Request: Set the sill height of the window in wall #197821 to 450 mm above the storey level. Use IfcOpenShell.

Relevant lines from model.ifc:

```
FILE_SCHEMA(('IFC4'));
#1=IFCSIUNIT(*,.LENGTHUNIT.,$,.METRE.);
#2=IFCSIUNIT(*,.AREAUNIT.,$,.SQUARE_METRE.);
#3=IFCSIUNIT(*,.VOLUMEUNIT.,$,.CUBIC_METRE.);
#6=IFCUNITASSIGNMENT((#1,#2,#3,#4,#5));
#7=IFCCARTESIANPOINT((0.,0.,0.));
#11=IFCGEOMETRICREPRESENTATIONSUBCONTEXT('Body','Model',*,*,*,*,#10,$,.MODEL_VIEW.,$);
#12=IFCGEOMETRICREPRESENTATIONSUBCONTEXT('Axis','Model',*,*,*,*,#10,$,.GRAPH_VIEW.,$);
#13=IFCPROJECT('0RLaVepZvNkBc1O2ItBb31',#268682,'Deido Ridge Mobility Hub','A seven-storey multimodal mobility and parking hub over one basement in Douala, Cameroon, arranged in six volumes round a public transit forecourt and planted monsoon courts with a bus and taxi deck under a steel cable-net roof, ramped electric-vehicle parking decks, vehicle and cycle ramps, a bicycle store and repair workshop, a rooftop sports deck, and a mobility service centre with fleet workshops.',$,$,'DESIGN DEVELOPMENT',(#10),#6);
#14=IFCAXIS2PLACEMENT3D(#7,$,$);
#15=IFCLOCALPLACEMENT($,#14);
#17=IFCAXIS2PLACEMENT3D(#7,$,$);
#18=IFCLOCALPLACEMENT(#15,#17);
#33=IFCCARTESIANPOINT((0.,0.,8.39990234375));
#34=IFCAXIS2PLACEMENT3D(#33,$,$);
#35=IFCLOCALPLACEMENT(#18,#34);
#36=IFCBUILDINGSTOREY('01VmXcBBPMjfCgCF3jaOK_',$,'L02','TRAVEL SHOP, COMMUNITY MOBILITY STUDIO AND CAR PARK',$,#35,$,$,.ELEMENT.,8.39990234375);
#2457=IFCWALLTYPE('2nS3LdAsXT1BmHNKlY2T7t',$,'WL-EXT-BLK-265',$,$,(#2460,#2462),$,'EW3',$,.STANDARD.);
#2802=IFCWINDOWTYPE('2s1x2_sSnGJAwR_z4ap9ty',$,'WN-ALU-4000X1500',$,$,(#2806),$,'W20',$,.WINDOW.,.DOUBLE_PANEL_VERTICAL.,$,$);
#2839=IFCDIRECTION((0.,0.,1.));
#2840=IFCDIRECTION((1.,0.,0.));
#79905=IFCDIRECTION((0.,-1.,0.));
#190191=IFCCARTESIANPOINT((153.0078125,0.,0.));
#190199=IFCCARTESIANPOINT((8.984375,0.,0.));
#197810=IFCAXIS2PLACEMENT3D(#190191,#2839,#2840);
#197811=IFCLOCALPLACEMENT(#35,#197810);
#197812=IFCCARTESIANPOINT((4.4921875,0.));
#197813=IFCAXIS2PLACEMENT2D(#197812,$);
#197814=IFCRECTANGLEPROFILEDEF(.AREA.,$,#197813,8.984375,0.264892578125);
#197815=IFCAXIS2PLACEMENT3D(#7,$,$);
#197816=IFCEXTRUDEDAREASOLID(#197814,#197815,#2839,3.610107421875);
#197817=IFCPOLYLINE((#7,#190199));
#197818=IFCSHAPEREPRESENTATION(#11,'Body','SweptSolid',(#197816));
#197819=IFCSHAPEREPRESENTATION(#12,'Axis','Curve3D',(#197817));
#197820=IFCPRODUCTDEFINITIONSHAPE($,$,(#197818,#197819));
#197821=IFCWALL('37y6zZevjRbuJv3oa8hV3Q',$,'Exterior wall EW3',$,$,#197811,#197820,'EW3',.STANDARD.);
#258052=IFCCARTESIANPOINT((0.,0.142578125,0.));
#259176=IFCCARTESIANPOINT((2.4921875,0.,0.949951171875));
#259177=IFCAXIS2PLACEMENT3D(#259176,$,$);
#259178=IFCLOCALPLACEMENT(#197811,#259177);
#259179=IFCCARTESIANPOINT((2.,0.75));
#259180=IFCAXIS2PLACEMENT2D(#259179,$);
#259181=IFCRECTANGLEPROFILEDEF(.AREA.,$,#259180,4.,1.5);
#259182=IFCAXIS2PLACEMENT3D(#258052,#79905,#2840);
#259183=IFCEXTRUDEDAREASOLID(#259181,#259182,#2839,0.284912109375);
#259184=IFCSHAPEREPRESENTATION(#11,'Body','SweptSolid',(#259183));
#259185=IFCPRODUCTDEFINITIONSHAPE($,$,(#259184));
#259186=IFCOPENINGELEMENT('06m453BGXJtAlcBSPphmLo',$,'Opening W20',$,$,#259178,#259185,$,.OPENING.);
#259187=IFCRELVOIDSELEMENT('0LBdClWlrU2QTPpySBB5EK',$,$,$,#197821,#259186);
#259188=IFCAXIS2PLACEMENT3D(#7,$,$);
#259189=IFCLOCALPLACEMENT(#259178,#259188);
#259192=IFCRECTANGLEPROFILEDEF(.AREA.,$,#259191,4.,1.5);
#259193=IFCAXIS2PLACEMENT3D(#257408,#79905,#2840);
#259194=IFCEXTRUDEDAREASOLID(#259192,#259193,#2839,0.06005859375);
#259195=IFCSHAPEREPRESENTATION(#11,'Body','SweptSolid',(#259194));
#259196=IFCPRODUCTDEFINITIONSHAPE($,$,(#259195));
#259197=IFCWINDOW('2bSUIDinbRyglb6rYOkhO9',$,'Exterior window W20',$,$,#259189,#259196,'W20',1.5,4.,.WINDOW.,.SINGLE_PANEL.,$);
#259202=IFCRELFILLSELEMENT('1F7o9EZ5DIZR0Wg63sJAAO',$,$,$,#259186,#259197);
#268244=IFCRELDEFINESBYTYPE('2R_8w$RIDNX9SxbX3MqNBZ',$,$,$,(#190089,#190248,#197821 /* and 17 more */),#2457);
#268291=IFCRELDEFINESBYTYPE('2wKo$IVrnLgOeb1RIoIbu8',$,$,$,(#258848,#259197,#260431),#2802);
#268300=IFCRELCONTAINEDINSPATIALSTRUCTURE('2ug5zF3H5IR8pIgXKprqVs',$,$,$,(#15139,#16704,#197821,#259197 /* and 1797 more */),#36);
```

```python
import numpy as np
import ifcopenshell
import ifcopenshell.api.geometry
import ifcopenshell.geom
import ifcopenshell.util.element
import ifcopenshell.util.placement
import ifcopenshell.util.shape
import ifcopenshell.util.unit

model = ifcopenshell.open("model.ifc")
unit_scale = ifcopenshell.util.unit.calculate_unit_scale(model)

window = model.by_guid("2bSUIDinbRyglb6rYOkhO9")
opening = window.FillsVoids[0].RelatingOpeningElement
storey = ifcopenshell.util.element.get_container(window, ifc_class="IfcBuildingStorey")
level = ifcopenshell.util.placement.get_local_placement(storey.ObjectPlacement)[2, 3]

# The opening's origin need not be at the sill, so measure its lowest point.
shape = ifcopenshell.geom.create_shape(ifcopenshell.geom.settings(), opening)
bottom = ifcopenshell.util.shape.get_shape_bottom_elevation(shape, shape.geometry) / unit_scale
dz = level + 0.45 - bottom

shift = np.array([0.0, 0.0, dz])
# The window is placed relative to its opening, so it follows when the opening moves.
matrix = ifcopenshell.util.placement.get_local_placement(opening.ObjectPlacement)
matrix[:3, 3] += shift
ifcopenshell.api.geometry.edit_object_placement(
    model, product=opening, matrix=matrix, is_si=False, should_transform_children=True
)

print(f"moved by {dz * unit_scale:+.3f} m")

model.write("model-out.ifc")
```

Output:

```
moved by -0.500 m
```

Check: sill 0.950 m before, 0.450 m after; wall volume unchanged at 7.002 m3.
